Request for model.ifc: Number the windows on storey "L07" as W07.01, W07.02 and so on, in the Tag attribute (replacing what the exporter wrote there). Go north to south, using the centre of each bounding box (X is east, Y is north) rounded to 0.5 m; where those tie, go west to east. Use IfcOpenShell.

First a look at what the model holds.

```python
import ifcopenshell
import ifcopenshell.util.element
import ifcopenshell.util.placement

model = ifcopenshell.open("model.ifc")
print(model.schema)
storey = next(s for s in model.by_type("IfcBuildingStorey") if s.Name == "L07")
windows = [e for e in ifcopenshell.util.element.get_decomposition(storey) if e.is_a("IfcWindow")]
for e in sorted(windows, key=lambda e: e.id()):
    origin = ifcopenshell.util.placement.get_local_placement(e.ObjectPlacement)[:3, 3]
    print(e.id(), e.Tag, e.Name, origin.round(2) + 0.0, sep=" | ")
```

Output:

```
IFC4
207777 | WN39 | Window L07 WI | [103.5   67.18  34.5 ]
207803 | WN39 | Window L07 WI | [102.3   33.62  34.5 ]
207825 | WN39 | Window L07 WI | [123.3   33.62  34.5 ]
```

```python
import ifcopenshell
import ifcopenshell.geom
import ifcopenshell.util.element
import ifcopenshell.util.shape

model = ifcopenshell.open("model.ifc")
settings = ifcopenshell.geom.settings()
settings.set("use-world-coords", True)


def centre(element):
    shape = ifcopenshell.geom.create_shape(settings, element)
    return ifcopenshell.util.shape.get_bbox_centroid(shape.geometry)


storey = next(s for s in model.by_type("IfcBuildingStorey") if s.Name == "L07")
windows = [e for e in ifcopenshell.util.element.get_decomposition(storey) if e.is_a("IfcWindow")]

# Insertion points can sit at a corner or the storey origin, so sort by the geometry (in metres).
centres = {e: centre(e) for e in windows}
windows.sort(key=lambda e: (-round(centres[e][1] / 0.5), centres[e][0]))

for i, e in enumerate(windows, start=1):
    number = f"W07.{i:02d}"
    e.Tag = number
    print(e.id(), number)

model.write("model_v2.ifc")
```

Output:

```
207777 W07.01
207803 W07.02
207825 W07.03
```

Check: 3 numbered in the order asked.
